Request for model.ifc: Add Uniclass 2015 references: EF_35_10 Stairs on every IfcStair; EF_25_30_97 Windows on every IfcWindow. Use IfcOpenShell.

First a look at what the model holds.

```python
import ifcopenshell

model = ifcopenshell.open("model.ifc")
print(model.schema)
print("classifications:", [c.Name for c in model.by_type("IfcClassification")])
for ifc_class in ("IfcDoor", "IfcRoof", "IfcStair", "IfcWall", "IfcWindow"):
    print(ifc_class, len(model.by_type(ifc_class)))
```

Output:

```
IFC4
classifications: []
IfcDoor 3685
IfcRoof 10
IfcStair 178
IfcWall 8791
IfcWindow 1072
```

```python
import ifcopenshell
import ifcopenshell.api.classification

model = ifcopenshell.open("model.ifc")

system = ifcopenshell.api.classification.add_classification(model, classification="Uniclass 2015")

codes = {
    "IfcStair": ("EF_35_10", "Stairs"),
    "IfcWindow": ("EF_25_30_97", "Windows"),
}
for ifc_class, (code, name) in codes.items():
    products = model.by_type(ifc_class)
    ifcopenshell.api.classification.add_reference(
        model, products=products, classification=system, identification=code, name=name
    )
    print(code, len(products))

model.write("model_updated.ifc")
```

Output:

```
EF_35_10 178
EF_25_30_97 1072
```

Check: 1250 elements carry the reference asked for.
